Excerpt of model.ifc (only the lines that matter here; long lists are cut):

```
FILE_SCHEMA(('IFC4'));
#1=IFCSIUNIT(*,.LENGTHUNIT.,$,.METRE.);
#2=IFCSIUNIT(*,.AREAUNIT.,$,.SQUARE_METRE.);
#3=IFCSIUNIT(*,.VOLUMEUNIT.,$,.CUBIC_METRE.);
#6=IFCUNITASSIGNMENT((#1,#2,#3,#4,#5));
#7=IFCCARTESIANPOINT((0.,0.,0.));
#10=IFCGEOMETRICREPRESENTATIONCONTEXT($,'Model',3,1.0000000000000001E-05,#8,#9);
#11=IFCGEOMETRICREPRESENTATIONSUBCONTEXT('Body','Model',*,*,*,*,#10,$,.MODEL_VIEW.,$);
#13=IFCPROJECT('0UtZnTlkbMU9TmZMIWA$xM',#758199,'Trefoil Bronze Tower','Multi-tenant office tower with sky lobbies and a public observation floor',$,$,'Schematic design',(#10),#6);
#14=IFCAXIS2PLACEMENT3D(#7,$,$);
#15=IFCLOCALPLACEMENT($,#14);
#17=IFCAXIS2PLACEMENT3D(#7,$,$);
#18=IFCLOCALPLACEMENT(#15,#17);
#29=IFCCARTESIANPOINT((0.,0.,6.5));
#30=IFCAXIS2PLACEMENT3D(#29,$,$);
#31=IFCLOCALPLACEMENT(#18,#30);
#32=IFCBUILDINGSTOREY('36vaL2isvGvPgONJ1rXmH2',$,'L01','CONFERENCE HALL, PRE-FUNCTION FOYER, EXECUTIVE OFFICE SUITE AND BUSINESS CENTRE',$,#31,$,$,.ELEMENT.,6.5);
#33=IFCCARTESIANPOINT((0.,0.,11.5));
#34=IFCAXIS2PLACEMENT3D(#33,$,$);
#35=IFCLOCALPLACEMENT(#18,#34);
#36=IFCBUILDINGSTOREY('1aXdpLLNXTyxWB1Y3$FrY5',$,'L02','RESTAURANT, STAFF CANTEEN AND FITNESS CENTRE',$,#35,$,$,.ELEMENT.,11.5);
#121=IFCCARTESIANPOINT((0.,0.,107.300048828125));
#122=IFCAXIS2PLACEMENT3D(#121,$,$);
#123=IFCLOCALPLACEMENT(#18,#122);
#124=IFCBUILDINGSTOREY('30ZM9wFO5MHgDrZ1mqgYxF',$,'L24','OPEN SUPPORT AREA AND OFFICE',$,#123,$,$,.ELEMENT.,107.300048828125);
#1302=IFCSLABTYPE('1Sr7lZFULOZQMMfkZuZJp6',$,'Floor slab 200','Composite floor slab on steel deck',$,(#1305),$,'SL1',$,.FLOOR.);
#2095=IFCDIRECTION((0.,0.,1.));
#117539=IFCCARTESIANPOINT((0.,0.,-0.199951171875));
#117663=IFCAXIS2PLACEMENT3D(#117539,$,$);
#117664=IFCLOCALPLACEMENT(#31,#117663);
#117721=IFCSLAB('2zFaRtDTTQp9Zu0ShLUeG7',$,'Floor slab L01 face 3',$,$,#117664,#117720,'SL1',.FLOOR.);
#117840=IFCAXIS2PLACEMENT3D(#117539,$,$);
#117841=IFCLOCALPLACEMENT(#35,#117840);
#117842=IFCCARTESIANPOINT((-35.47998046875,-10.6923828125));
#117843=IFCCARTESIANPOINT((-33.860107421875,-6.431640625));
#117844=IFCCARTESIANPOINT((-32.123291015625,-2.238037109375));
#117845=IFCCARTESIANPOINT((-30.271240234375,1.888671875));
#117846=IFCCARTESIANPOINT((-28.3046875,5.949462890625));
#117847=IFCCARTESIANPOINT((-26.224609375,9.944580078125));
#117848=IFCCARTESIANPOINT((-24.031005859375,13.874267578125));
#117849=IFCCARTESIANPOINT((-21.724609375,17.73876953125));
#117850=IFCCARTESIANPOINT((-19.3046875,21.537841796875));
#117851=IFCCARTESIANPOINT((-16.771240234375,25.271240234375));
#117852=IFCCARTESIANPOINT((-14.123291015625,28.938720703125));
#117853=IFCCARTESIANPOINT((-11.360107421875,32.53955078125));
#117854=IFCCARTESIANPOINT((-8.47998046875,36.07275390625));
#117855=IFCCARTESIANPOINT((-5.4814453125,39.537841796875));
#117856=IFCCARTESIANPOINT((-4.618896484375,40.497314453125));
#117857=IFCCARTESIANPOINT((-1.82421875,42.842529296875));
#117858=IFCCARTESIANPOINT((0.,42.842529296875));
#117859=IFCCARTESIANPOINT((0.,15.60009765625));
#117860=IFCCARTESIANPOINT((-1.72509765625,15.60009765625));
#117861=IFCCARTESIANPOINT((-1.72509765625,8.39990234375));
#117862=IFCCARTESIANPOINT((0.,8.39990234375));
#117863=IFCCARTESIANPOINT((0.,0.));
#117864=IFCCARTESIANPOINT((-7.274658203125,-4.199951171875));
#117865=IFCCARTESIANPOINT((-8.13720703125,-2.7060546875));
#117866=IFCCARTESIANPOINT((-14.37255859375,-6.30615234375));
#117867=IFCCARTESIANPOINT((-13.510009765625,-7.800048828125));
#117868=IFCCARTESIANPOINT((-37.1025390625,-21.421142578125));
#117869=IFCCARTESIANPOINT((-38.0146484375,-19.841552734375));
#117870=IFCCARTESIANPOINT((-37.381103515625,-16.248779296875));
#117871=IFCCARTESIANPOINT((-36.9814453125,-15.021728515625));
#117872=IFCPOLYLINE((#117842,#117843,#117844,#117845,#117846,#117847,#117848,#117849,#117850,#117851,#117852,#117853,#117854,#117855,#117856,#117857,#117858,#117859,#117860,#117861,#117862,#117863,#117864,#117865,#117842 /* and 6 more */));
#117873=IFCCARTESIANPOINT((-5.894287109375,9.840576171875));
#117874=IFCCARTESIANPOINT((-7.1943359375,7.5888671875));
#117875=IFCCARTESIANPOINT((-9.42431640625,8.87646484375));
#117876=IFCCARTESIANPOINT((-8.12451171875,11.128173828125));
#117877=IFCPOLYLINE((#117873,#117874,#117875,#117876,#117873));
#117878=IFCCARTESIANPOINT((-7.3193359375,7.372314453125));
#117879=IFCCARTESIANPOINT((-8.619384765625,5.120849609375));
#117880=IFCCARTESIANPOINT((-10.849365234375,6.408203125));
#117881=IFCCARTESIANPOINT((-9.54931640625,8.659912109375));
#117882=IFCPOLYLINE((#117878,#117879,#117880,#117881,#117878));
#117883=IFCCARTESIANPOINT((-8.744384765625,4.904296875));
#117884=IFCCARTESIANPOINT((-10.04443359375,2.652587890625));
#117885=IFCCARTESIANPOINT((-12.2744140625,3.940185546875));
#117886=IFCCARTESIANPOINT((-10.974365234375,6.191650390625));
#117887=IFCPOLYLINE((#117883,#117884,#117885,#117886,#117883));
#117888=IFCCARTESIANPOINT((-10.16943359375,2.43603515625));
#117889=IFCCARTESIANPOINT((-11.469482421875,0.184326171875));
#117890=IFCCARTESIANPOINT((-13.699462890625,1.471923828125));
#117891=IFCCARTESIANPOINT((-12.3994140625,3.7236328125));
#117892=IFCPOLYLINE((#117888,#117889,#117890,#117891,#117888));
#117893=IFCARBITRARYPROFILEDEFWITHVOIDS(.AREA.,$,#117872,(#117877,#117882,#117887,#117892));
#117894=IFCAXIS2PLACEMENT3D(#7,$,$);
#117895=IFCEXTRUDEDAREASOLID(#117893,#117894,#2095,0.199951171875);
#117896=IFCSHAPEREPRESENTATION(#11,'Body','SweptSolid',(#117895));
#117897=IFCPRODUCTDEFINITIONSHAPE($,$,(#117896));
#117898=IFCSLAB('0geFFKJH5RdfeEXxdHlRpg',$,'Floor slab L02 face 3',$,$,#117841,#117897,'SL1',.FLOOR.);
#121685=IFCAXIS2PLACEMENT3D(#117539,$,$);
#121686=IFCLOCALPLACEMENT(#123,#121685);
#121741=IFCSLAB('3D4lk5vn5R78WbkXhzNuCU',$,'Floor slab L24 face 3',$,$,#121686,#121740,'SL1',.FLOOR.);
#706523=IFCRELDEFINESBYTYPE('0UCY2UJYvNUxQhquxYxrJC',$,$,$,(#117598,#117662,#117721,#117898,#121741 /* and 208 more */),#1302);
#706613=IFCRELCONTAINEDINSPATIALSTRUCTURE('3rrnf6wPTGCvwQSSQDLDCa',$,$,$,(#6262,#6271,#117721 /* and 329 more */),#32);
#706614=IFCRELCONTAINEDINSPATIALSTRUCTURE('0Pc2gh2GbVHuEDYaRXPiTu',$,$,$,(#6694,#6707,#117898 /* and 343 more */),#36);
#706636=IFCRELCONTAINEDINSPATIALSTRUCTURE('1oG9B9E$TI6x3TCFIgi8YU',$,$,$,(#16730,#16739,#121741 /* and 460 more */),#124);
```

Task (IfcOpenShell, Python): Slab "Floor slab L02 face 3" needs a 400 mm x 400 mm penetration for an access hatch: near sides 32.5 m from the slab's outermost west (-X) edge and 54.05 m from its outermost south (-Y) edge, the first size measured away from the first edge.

```python
import numpy as np
import ifcopenshell
import ifcopenshell.api.feature
import ifcopenshell.api.geometry
import ifcopenshell.api.root
import ifcopenshell.geom
import ifcopenshell.util.placement
import ifcopenshell.util.representation
import ifcopenshell.util.shape
import ifcopenshell.util.unit

model = ifcopenshell.open("model.ifc")
unit_scale = ifcopenshell.util.unit.calculate_unit_scale(model)
settings = ifcopenshell.geom.settings()


def volume(element):
    """Net volume in cubic metres, openings subtracted."""
    shape = ifcopenshell.geom.create_shape(settings, element)
    return ifcopenshell.util.shape.get_volume(shape.geometry)


slab = model.by_guid("0geFFKJH5RdfeEXxdHlRpg")
before = volume(slab)

# Extent in the slab's own axes, in metres. The edges named are its -X and -Y sides.
slab_shape = ifcopenshell.geom.create_shape(settings, slab)
vertices = ifcopenshell.util.shape.get_vertices(slab_shape.geometry)
x_min, y_min, bottom = vertices.min(axis=0)
top = vertices[:, 2].max()

opening = ifcopenshell.api.root.create_entity(model, ifc_class="IfcOpeningElement", name="Access hatch opening", predefined_type="OPENING")
context = ifcopenshell.util.representation.get_context(model, "Model", "Body", "MODEL_VIEW")
width, depth = 0.4, 0.4
outline = [(0.0, 0.0), (width, 0.0), (width, depth), (0.0, depth), (0.0, 0.0)]
# Overshoot both faces by 50 mm so the cut is clean.
shape = ifcopenshell.api.geometry.add_slab_representation(
    model, context=context, depth=top - bottom + 0.1, polyline=outline
)
ifcopenshell.api.geometry.assign_representation(model, product=opening, representation=shape)

matrix = ifcopenshell.util.placement.get_local_placement(slab.ObjectPlacement)
matrix[:, 3] = matrix @ np.append(np.array([x_min + 32.5, y_min + 54.05, bottom - 0.05]) / unit_scale, 1.0)
ifcopenshell.api.geometry.edit_object_placement(model, product=opening, matrix=matrix, is_si=False)
ifcopenshell.api.feature.add_feature(model, feature=opening, element=slab)

after = volume(slab)

print(f"slab volume {before:.3f} -> {after:.3f} m3")

model.write("model_edited.ifc")
```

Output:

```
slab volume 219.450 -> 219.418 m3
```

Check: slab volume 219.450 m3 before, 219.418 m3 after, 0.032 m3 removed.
